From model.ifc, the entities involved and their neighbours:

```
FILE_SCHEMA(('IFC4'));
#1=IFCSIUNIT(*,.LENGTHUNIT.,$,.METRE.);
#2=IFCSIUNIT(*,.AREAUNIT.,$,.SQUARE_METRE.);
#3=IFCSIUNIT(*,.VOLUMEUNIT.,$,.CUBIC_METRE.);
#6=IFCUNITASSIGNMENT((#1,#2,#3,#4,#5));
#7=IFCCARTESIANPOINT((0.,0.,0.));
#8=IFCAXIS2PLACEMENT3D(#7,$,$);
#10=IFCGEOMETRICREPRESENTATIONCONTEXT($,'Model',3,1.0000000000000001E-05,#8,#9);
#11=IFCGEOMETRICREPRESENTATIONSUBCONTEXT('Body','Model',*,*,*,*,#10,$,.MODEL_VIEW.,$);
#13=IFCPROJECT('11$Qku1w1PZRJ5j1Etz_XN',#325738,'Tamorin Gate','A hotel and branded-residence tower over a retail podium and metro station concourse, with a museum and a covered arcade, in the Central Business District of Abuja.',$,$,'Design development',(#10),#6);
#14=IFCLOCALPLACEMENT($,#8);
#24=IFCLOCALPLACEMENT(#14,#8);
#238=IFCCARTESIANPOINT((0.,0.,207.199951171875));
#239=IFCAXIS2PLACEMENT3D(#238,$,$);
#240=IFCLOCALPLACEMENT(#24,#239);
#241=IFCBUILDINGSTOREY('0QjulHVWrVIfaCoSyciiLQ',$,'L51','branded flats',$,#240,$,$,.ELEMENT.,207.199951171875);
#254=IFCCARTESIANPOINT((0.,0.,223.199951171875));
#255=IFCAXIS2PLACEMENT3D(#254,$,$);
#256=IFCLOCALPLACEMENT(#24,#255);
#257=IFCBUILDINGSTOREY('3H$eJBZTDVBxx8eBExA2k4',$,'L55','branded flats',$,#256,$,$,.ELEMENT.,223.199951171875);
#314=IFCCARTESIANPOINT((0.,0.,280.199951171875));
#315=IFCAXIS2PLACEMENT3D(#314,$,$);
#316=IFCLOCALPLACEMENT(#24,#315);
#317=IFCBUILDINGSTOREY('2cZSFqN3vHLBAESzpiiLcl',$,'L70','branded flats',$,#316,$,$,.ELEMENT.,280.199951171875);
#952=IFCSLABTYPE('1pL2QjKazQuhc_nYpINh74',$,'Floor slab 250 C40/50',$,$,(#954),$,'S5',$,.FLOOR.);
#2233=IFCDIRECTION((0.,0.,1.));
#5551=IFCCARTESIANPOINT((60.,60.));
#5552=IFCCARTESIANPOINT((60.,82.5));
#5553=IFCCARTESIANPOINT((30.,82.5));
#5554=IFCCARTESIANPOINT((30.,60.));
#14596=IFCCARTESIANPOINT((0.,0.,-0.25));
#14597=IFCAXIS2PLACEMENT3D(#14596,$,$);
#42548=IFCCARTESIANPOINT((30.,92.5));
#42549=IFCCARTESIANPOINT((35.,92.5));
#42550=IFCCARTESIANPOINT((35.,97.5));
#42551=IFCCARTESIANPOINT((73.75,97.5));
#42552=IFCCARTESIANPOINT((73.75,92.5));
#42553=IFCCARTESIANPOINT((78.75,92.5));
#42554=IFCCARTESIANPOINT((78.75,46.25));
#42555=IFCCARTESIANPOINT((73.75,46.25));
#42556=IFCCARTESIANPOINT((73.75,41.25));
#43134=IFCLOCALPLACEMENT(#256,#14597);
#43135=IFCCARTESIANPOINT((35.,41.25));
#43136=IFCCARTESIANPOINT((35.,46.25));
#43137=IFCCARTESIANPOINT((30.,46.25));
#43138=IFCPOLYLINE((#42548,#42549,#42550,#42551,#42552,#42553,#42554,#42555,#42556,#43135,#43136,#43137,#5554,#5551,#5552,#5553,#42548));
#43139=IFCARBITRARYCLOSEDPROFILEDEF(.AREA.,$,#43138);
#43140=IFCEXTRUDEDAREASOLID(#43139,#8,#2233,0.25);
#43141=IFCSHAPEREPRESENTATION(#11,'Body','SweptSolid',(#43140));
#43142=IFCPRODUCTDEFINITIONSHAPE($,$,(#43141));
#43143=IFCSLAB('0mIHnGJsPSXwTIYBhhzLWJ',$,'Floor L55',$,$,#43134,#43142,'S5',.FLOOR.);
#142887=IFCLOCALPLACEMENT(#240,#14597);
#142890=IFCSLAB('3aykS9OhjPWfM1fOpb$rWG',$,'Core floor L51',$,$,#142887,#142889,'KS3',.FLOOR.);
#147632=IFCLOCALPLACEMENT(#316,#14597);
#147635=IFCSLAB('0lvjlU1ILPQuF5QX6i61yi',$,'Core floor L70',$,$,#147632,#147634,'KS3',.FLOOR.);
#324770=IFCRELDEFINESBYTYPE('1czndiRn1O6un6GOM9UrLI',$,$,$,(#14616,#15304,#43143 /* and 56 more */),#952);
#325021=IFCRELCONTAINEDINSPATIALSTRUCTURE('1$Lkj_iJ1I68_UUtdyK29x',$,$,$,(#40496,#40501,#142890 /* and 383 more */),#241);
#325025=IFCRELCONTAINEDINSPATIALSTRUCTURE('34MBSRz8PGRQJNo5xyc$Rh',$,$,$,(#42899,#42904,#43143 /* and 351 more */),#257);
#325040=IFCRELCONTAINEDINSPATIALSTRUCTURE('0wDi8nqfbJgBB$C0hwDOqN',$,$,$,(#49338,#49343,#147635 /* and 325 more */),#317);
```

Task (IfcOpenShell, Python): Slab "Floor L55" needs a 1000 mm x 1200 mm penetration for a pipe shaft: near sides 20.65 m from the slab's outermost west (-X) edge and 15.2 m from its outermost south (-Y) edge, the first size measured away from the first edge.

```python
import numpy as np
import ifcopenshell
import ifcopenshell.api.feature
import ifcopenshell.api.geometry
import ifcopenshell.api.root
import ifcopenshell.geom
import ifcopenshell.util.placement
import ifcopenshell.util.representation
import ifcopenshell.util.shape
import ifcopenshell.util.unit

model = ifcopenshell.open("model.ifc")
unit_scale = ifcopenshell.util.unit.calculate_unit_scale(model)
settings = ifcopenshell.geom.settings()


def volume(element):
    """Net volume in cubic metres, openings subtracted."""
    shape = ifcopenshell.geom.create_shape(settings, element)
    return ifcopenshell.util.shape.get_volume(shape.geometry)


slab = model.by_guid("0mIHnGJsPSXwTIYBhhzLWJ")
before = volume(slab)

# Extent in the slab's own axes, in metres. The edges named are its -X and -Y sides.
slab_shape = ifcopenshell.geom.create_shape(settings, slab)
vertices = ifcopenshell.util.shape.get_vertices(slab_shape.geometry)
x_min, y_min, bottom = vertices.min(axis=0)
top = vertices[:, 2].max()

opening = ifcopenshell.api.root.create_entity(model, ifc_class="IfcOpeningElement", name="Pipe shaft opening", predefined_type="OPENING")
context = ifcopenshell.util.representation.get_context(model, "Model", "Body", "MODEL_VIEW")
width, depth = 1, 1.2
outline = [(0.0, 0.0), (width, 0.0), (width, depth), (0.0, depth), (0.0, 0.0)]
# Overshoot both faces by 50 mm so the cut is clean.
shape = ifcopenshell.api.geometry.add_slab_representation(
    model, context=context, depth=top - bottom + 0.1, polyline=outline
)
ifcopenshell.api.geometry.assign_representation(model, product=opening, representation=shape)

matrix = ifcopenshell.util.placement.get_local_placement(slab.ObjectPlacement)
matrix[:, 3] = matrix @ np.append(np.array([x_min + 20.65, y_min + 15.2, bottom - 0.05]) / unit_scale, 1.0)
ifcopenshell.api.geometry.edit_object_placement(model, product=opening, matrix=matrix, is_si=False)
ifcopenshell.api.feature.add_feature(model, feature=opening, element=slab)

after = volume(slab)

print(f"slab volume {before:.3f} -> {after:.3f} m3")

model.write("model-out.ifc")
```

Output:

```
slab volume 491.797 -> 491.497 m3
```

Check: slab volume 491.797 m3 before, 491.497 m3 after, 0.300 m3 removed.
